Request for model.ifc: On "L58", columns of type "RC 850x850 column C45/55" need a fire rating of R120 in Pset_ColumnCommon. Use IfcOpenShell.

First a look at what the model holds.

```python
import ifcopenshell
import ifcopenshell.util.element

model = ifcopenshell.open("model.ifc")
print(model.schema)
storey = next(s for s in model.by_type("IfcBuildingStorey") if s.Name == "L58")
columns = [e for e in ifcopenshell.util.element.get_decomposition(storey) if e.is_a("IfcColumn")]
seen = {}
for e in columns:
    element_type = ifcopenshell.util.element.get_type(e)
    key = (element_type.Name if element_type != e and element_type else None, ifcopenshell.util.element.get_pset(e, "Pset_ColumnCommon", "FireRating"))
    seen[key] = seen.get(key, 0) + 1
for (name, value), count in sorted(seen.items(), key=str):
    print(count, "x", name, "|", value)
```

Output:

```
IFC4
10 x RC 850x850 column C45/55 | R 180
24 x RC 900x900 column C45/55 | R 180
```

```python
import ifcopenshell
import ifcopenshell.api.pset
import ifcopenshell.util.element

model = ifcopenshell.open("model.ifc")

storey = next(s for s in model.by_type("IfcBuildingStorey") if s.Name == "L58")
columns = [e for e in ifcopenshell.util.element.get_decomposition(storey) if e.is_a("IfcColumn")]

count = 0
for e in columns:
    element_type = ifcopenshell.util.element.get_type(e)
    if element_type in (None, e) or element_type.Name != "RC 850x850 column C45/55":
        continue
    found = ifcopenshell.util.element.get_pset(e, "Pset_ColumnCommon", should_inherit=False)
    if found:
        pset = model.by_id(found["id"])
        if len(ifcopenshell.util.element.get_elements_by_pset(pset)) > 1:
            pset = ifcopenshell.api.pset.unshare_pset(model, products=[e], pset=pset)[0]
    else:
        pset = ifcopenshell.api.pset.add_pset(model, product=e, name="Pset_ColumnCommon")
    ifcopenshell.api.pset.edit_pset(model, pset=pset, properties={"FireRating": "R120"})
    count += 1

print(count, "columns updated")

model.write("model_edited.ifc")
```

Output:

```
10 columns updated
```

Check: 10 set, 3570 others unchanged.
